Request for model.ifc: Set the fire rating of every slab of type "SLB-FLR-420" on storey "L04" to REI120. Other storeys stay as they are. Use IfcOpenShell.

First a look at what the model holds.

```python
import ifcopenshell
import ifcopenshell.util.element

model = ifcopenshell.open("model.ifc")
print(model.schema)
storey = next(s for s in model.by_type("IfcBuildingStorey") if s.Name == "L04")
slabs = [e for e in ifcopenshell.util.element.get_decomposition(storey) if e.is_a("IfcSlab")]
seen = {}
for e in slabs:
    element_type = ifcopenshell.util.element.get_type(e)
    key = (element_type.Name if element_type != e and element_type else None, ifcopenshell.util.element.get_pset(e, "Pset_SlabCommon", "FireRating"))
    seen[key] = seen.get(key, 0) + 1
for (name, value), count in sorted(seen.items(), key=str):
    print(count, "x", name, "|", value)
```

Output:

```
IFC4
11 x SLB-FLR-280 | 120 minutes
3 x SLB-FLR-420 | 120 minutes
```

```python
import ifcopenshell
import ifcopenshell.api.pset
import ifcopenshell.util.element

model = ifcopenshell.open("model.ifc")

storey = next(s for s in model.by_type("IfcBuildingStorey") if s.Name == "L04")
slabs = [e for e in ifcopenshell.util.element.get_decomposition(storey) if e.is_a("IfcSlab")]

count = 0
for e in slabs:
    element_type = ifcopenshell.util.element.get_type(e)
    if element_type in (None, e) or element_type.Name != "SLB-FLR-420":
        continue
    # add_pset returns the element's existing set when there is one.
    pset = ifcopenshell.api.pset.add_pset(model, product=e, name="Pset_SlabCommon")
    ifcopenshell.api.pset.edit_pset(model, pset=pset, properties={"FireRating": "REI120"})
    count += 1

print(count, "slabs updated")

model.write("model-out.ifc")
```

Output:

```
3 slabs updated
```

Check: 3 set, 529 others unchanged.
